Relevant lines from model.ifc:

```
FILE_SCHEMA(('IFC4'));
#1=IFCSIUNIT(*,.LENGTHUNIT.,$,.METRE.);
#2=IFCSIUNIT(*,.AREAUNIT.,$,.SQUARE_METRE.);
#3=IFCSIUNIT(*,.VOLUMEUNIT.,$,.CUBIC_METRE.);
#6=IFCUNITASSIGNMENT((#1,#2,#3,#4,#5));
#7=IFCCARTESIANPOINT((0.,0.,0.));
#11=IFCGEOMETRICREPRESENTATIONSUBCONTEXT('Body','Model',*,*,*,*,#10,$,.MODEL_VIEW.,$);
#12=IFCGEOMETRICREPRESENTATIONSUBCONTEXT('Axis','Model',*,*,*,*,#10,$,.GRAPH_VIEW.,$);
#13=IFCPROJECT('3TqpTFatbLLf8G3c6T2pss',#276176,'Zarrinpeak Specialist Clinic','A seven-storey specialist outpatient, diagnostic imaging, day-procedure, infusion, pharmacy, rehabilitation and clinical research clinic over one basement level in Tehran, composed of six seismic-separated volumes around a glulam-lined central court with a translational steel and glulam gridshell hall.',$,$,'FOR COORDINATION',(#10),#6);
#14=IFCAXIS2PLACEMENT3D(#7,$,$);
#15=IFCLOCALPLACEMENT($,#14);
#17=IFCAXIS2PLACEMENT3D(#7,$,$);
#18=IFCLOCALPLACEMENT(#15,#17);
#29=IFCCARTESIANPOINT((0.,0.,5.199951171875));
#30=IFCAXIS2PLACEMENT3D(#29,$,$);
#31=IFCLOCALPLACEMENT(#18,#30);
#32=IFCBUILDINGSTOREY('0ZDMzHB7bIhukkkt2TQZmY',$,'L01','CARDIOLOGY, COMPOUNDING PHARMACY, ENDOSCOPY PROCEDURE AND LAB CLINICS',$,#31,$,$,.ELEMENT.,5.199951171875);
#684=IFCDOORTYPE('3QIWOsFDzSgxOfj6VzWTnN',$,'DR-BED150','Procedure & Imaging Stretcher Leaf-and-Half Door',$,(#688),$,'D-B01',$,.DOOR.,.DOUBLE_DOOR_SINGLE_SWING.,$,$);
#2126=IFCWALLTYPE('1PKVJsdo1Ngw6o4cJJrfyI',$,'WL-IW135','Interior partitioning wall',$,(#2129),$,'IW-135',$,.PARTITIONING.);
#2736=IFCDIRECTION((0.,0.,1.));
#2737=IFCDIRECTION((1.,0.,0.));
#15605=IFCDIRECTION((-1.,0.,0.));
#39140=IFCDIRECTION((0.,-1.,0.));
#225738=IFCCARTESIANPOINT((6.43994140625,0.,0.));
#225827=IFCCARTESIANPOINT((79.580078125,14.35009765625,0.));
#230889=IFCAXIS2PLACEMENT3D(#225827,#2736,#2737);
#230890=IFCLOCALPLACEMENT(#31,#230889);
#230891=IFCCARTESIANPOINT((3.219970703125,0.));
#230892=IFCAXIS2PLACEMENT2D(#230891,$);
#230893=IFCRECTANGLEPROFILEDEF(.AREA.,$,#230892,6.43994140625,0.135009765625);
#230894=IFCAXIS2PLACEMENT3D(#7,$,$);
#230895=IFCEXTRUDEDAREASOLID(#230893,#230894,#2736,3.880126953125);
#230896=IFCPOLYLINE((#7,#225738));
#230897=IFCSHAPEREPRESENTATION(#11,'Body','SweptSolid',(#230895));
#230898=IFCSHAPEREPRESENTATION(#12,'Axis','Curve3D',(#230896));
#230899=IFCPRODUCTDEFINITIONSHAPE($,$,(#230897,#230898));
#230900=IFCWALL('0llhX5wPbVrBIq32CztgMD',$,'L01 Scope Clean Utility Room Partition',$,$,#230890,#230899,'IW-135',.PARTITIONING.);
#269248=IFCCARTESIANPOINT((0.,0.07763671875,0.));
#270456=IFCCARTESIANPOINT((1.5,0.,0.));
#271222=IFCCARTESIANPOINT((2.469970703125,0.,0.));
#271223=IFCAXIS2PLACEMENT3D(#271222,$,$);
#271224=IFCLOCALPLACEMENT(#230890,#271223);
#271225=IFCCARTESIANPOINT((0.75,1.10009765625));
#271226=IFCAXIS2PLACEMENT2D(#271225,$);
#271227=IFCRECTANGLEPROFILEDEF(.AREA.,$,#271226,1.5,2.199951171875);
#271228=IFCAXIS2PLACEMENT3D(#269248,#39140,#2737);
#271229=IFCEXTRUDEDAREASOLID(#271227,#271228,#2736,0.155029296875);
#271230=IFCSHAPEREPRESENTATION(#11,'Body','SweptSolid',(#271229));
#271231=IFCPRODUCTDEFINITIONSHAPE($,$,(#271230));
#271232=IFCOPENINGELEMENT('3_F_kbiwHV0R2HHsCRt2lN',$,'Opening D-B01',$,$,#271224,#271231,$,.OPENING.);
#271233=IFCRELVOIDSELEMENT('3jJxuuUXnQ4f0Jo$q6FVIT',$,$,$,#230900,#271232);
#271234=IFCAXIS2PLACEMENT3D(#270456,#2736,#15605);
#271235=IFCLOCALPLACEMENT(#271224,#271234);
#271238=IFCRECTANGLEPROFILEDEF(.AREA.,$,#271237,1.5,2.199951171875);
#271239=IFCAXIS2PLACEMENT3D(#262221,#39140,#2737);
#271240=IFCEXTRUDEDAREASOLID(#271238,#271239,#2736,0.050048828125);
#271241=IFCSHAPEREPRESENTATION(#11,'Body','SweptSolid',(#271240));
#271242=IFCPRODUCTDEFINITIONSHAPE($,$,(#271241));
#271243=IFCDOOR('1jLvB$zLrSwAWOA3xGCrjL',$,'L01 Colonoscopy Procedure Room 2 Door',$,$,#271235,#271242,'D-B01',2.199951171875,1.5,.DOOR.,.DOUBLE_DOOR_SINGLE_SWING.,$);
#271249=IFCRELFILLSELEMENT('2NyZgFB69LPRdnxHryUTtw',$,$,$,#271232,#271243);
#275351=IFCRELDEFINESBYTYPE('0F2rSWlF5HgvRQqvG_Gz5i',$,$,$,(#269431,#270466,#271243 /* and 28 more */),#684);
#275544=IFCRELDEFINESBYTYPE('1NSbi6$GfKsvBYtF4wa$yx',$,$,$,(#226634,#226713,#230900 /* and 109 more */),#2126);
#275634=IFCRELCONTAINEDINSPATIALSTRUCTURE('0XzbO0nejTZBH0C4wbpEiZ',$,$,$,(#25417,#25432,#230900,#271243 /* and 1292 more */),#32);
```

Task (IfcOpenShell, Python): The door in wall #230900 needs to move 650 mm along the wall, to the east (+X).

```python
import ifcopenshell
import ifcopenshell.api.geometry
import ifcopenshell.util.placement

model = ifcopenshell.open("model.ifc")

door = model.by_guid("1jLvB$zLrSwAWOA3xGCrjL")
opening = door.FillsVoids[0].RelatingOpeningElement
wall = opening.VoidsElements[0].RelatingBuildingElement

wall_matrix = ifcopenshell.util.placement.get_local_placement(wall.ObjectPlacement)
shift = wall_matrix[:3, 0] * 0.65
before = ifcopenshell.util.placement.get_local_placement(door.ObjectPlacement)[:3, 3].copy()

# The door is placed relative to its opening, so it follows when the opening moves.
matrix = ifcopenshell.util.placement.get_local_placement(opening.ObjectPlacement)
matrix[:3, 3] += shift
ifcopenshell.api.geometry.edit_object_placement(
    model, product=opening, matrix=matrix, is_si=False, should_transform_children=True
)

after = ifcopenshell.util.placement.get_local_placement(door.ObjectPlacement)[:3, 3]
print("door moved by", (after - before).round(3) + 0.0)

model.write("model_updated.ifc")
```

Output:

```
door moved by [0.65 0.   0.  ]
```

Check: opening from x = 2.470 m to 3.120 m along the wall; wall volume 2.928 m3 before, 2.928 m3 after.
